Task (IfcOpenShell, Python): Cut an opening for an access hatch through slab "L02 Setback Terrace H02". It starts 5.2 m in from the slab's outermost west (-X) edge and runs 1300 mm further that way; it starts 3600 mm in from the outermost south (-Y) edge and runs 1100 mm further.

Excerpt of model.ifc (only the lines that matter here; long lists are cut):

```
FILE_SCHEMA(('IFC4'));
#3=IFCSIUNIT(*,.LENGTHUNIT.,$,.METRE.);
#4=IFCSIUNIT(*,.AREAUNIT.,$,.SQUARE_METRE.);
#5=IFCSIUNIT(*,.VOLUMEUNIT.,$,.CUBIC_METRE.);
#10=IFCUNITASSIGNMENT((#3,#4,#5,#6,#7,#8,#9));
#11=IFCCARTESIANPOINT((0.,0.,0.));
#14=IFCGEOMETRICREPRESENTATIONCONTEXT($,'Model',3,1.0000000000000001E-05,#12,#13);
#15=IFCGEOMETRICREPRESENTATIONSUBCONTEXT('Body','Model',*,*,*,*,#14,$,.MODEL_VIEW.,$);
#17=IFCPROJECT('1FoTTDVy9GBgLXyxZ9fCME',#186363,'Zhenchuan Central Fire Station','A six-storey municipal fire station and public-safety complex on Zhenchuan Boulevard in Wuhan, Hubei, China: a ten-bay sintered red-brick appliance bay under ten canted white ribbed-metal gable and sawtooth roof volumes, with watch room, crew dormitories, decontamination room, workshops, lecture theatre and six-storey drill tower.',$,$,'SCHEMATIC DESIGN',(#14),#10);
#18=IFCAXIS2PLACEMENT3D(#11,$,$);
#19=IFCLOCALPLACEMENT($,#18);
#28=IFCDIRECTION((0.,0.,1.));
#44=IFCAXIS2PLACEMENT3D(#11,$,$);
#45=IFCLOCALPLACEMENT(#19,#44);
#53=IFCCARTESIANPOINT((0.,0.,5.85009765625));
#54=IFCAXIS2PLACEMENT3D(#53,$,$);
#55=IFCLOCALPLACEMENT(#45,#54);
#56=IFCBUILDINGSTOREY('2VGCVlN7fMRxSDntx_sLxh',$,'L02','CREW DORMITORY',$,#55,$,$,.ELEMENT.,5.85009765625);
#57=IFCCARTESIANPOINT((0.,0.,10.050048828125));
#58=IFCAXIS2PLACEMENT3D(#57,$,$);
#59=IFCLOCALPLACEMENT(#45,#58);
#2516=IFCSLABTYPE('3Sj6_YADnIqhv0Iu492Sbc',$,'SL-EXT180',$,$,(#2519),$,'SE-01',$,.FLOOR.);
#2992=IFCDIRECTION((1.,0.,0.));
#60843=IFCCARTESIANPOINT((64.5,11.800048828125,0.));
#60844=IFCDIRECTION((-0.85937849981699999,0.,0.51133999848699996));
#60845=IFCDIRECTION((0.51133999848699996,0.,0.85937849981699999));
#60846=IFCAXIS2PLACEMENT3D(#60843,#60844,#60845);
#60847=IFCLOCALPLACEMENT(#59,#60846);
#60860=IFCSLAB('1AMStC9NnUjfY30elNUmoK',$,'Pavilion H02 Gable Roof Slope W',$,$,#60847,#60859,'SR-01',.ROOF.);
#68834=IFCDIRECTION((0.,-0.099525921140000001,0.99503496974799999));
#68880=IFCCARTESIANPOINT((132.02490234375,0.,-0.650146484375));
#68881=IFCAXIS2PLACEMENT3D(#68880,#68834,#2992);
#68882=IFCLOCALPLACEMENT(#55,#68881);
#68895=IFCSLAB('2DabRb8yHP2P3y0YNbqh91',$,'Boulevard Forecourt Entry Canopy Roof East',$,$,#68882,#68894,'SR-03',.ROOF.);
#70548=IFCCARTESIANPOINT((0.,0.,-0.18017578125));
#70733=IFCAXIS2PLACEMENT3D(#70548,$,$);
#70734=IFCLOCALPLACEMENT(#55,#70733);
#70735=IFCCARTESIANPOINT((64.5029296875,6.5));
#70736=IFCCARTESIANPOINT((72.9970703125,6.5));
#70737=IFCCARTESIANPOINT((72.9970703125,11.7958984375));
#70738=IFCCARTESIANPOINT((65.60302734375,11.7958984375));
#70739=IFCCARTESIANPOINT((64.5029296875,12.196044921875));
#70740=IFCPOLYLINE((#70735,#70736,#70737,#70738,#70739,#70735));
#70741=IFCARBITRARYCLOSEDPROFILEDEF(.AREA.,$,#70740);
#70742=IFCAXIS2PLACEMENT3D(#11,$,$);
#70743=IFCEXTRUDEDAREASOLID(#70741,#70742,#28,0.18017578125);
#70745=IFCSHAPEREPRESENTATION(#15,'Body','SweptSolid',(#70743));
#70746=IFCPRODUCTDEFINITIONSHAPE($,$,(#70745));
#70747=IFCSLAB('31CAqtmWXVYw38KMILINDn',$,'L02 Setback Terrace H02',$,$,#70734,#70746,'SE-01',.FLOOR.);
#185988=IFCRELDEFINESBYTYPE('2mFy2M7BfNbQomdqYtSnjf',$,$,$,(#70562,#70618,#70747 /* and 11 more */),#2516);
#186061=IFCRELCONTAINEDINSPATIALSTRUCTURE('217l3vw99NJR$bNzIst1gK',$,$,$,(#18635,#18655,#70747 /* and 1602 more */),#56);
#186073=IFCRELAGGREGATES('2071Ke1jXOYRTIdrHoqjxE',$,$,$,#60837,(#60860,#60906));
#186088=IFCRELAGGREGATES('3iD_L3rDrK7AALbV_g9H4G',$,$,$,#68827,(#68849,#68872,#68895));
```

```python
import numpy as np
import ifcopenshell
import ifcopenshell.api.feature
import ifcopenshell.api.geometry
import ifcopenshell.api.root
import ifcopenshell.geom
import ifcopenshell.util.placement
import ifcopenshell.util.representation
import ifcopenshell.util.shape
import ifcopenshell.util.unit

model = ifcopenshell.open("model.ifc")
unit_scale = ifcopenshell.util.unit.calculate_unit_scale(model)
settings = ifcopenshell.geom.settings()


def volume(element):
    """Net volume in cubic metres, openings subtracted."""
    shape = ifcopenshell.geom.create_shape(settings, element)
    return ifcopenshell.util.shape.get_volume(shape.geometry)


slab = model.by_guid("31CAqtmWXVYw38KMILINDn")
before = volume(slab)

# Extent in the slab's own axes, in metres. The edges named are its -X and -Y sides.
slab_shape = ifcopenshell.geom.create_shape(settings, slab)
vertices = ifcopenshell.util.shape.get_vertices(slab_shape.geometry)
x_min, y_min, bottom = vertices.min(axis=0)
top = vertices[:, 2].max()

opening = ifcopenshell.api.root.create_entity(model, ifc_class="IfcOpeningElement", name="Access hatch opening", predefined_type="OPENING")
context = ifcopenshell.util.representation.get_context(model, "Model", "Body", "MODEL_VIEW")
width, depth = 1.3, 1.1
outline = [(0.0, 0.0), (width, 0.0), (width, depth), (0.0, depth), (0.0, 0.0)]
# Overshoot both faces by 50 mm so the cut is clean.
shape = ifcopenshell.api.geometry.add_slab_representation(
    model, context=context, depth=top - bottom + 0.1, polyline=outline
)
ifcopenshell.api.geometry.assign_representation(model, product=opening, representation=shape)

matrix = ifcopenshell.util.placement.get_local_placement(slab.ObjectPlacement)
matrix[:, 3] = matrix @ np.append(np.array([x_min + 5.2, y_min + 3.6, bottom - 0.05]) / unit_scale, 1.0)
ifcopenshell.api.geometry.edit_object_placement(model, product=opening, matrix=matrix, is_si=False)
ifcopenshell.api.feature.add_feature(model, feature=opening, element=slab)

after = volume(slab)

print(f"slab volume {before:.3f} -> {after:.3f} m3")

model.write("model_v2.ifc")
```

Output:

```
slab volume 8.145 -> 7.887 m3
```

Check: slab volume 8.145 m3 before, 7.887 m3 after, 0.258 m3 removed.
